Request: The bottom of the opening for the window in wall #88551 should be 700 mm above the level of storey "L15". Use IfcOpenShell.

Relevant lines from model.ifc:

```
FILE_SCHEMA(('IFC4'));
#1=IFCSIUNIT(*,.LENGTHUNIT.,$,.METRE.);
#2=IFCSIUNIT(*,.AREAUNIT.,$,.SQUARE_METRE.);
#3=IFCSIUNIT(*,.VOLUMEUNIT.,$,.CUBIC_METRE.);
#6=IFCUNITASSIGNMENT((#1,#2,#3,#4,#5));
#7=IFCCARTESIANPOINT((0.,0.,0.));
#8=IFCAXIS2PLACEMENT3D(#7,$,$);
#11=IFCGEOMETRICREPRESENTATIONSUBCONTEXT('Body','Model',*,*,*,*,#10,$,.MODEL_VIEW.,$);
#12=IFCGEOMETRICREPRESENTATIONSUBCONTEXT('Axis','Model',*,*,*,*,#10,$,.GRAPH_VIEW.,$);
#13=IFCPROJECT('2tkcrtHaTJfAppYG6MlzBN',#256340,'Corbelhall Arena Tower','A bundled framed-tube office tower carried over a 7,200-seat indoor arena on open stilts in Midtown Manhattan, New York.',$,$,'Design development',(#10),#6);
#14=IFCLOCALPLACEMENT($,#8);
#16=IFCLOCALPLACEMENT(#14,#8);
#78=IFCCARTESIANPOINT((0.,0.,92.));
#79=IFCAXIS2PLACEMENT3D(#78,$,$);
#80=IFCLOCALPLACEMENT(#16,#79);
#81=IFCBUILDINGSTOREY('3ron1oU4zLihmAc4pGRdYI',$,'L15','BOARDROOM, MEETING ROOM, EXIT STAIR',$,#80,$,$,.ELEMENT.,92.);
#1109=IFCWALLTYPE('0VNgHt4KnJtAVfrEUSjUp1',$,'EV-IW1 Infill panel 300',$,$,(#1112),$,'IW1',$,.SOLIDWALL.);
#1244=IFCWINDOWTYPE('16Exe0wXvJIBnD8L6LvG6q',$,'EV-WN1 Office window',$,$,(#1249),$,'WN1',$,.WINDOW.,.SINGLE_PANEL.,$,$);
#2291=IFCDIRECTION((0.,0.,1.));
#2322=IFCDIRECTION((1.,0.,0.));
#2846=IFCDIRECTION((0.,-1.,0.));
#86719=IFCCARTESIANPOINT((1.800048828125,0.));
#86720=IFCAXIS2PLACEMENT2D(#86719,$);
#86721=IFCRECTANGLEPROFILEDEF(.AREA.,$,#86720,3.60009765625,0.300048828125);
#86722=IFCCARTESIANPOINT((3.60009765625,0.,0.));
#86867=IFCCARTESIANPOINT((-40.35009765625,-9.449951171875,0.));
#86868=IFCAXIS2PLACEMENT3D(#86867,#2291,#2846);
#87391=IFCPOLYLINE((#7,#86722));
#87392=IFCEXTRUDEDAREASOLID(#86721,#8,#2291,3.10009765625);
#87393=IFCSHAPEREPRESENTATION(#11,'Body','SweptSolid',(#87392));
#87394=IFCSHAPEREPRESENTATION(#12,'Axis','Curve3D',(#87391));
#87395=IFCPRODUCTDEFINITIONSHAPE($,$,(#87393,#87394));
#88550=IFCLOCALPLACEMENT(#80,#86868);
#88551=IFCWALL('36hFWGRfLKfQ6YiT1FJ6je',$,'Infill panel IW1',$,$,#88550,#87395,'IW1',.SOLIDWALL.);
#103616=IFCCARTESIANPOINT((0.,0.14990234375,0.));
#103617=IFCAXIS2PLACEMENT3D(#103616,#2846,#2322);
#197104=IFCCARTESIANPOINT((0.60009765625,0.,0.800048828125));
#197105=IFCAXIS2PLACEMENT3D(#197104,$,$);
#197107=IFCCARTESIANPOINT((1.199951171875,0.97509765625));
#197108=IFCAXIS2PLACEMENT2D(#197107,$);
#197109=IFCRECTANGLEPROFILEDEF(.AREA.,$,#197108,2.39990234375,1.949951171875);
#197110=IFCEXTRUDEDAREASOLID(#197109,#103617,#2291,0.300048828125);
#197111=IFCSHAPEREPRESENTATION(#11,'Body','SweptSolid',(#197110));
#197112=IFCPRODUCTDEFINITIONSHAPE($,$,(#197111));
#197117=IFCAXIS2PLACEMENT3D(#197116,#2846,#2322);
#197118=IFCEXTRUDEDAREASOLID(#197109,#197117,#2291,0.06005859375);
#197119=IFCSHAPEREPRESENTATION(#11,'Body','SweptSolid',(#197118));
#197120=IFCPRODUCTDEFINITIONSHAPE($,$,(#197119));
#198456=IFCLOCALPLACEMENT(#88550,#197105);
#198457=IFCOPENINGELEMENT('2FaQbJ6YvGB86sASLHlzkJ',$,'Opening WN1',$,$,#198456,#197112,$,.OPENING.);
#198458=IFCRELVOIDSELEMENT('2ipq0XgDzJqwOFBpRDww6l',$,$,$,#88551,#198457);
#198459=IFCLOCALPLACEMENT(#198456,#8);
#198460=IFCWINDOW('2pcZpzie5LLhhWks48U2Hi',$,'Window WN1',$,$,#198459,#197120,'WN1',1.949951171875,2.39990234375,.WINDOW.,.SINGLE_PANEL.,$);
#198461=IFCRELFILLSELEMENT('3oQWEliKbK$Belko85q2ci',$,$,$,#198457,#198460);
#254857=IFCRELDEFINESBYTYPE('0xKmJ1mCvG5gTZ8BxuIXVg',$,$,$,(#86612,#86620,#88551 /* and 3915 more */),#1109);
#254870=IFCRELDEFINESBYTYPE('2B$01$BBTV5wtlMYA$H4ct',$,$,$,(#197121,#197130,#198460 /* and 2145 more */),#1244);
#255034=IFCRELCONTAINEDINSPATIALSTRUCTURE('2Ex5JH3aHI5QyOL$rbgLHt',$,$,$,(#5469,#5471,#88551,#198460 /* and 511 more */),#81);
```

```python
import numpy as np
import ifcopenshell
import ifcopenshell.api.geometry
import ifcopenshell.geom
import ifcopenshell.util.element
import ifcopenshell.util.placement
import ifcopenshell.util.shape
import ifcopenshell.util.unit

model = ifcopenshell.open("model.ifc")
unit_scale = ifcopenshell.util.unit.calculate_unit_scale(model)

window = model.by_id(198460)
opening = window.FillsVoids[0].RelatingOpeningElement
storey = ifcopenshell.util.element.get_container(window, ifc_class="IfcBuildingStorey")
level = ifcopenshell.util.placement.get_local_placement(storey.ObjectPlacement)[2, 3]

# The opening's origin need not be at the sill, so measure its lowest point.
shape = ifcopenshell.geom.create_shape(ifcopenshell.geom.settings(), opening)
bottom = ifcopenshell.util.shape.get_shape_bottom_elevation(shape, shape.geometry) / unit_scale
dz = level + 0.7 / unit_scale - bottom

shift = np.array([0.0, 0.0, dz])
# The window is placed relative to its opening, so it follows when the opening moves.
matrix = ifcopenshell.util.placement.get_local_placement(opening.ObjectPlacement)
matrix[:3, 3] += shift
ifcopenshell.api.geometry.edit_object_placement(
    model, product=opening, matrix=matrix, is_si=False, should_transform_children=True
)

print(f"moved by {dz * unit_scale:+.3f} m")

model.write("model_v2.ifc")
```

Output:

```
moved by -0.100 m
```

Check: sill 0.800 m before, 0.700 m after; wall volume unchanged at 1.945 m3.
